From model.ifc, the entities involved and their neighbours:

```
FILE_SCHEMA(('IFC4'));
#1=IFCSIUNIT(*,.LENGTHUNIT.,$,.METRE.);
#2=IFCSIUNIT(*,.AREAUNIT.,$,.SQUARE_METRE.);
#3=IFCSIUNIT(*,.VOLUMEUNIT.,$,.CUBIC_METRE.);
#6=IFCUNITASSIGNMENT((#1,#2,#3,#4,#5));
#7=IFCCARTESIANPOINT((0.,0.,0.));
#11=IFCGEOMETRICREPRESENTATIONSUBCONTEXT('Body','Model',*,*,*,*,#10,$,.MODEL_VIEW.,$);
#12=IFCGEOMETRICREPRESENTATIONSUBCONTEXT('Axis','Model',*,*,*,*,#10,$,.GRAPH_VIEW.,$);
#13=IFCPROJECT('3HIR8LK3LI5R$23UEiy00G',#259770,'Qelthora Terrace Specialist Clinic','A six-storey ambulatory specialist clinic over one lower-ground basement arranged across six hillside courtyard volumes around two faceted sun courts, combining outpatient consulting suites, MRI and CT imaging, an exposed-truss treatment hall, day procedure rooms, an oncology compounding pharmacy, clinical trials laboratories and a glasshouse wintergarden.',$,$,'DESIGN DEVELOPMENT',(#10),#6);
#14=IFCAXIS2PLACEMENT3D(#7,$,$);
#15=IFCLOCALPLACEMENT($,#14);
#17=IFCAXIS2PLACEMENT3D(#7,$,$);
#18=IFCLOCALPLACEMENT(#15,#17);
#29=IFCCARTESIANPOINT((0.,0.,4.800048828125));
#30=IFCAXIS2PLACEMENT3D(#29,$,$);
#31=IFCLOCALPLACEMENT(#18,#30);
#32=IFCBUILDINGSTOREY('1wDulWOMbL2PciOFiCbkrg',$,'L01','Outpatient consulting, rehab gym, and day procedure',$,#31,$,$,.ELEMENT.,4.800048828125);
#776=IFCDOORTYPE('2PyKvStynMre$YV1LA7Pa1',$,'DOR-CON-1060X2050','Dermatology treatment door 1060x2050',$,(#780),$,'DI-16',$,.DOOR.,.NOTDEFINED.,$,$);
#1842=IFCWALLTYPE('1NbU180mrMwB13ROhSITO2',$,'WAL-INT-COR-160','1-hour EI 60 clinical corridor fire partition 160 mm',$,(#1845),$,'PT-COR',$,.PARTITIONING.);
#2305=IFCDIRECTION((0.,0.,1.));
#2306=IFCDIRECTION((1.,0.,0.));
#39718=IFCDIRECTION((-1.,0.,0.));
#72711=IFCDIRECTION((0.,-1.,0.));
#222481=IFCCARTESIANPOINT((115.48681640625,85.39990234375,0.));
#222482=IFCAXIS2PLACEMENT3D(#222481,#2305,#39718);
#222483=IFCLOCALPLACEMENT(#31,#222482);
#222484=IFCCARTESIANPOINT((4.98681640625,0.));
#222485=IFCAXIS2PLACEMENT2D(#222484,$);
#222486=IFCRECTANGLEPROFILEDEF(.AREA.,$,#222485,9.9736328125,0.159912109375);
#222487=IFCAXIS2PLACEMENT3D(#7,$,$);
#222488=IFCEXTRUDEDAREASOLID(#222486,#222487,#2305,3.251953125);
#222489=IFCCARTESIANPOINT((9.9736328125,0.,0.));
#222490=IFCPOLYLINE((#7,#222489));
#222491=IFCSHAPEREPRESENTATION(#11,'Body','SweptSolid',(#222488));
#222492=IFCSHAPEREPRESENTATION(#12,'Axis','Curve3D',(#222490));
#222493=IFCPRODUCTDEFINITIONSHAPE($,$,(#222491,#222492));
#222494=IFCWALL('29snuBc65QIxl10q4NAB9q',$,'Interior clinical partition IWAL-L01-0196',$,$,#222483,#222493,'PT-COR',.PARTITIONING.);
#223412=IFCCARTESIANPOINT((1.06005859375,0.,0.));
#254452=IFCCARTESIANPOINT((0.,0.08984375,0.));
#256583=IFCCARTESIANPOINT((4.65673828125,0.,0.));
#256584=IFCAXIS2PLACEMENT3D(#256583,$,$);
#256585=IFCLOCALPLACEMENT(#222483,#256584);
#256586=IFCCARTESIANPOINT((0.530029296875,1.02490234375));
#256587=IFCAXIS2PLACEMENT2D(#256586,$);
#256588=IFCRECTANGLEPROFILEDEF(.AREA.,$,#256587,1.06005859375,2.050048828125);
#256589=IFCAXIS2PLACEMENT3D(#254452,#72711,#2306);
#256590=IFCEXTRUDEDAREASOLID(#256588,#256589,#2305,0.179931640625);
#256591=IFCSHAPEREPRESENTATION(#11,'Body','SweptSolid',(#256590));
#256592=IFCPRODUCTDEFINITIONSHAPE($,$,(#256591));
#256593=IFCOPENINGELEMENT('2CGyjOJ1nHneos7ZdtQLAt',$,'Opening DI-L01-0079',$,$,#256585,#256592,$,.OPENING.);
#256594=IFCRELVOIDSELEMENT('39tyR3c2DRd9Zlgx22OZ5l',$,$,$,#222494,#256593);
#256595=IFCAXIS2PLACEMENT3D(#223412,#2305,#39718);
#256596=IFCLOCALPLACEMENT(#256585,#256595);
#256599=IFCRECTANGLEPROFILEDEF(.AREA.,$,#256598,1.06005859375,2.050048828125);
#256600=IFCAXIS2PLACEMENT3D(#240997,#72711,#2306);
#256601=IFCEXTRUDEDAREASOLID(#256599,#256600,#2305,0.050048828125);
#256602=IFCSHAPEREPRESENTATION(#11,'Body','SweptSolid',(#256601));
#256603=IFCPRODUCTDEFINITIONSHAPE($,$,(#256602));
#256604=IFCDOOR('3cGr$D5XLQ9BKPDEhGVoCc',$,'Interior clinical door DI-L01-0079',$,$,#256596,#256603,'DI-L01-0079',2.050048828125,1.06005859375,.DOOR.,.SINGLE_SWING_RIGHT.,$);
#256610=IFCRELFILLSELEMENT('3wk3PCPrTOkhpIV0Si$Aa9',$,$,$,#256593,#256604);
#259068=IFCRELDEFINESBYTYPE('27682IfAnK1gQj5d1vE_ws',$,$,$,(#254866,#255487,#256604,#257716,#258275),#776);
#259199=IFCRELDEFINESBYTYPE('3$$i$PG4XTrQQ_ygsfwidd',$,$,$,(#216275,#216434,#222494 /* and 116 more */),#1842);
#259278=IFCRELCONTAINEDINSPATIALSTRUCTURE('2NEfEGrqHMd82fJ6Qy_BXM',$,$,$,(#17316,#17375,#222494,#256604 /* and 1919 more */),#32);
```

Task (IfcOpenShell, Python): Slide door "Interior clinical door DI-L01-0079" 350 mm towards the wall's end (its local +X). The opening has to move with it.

```python
import ifcopenshell
import ifcopenshell.api.geometry
import ifcopenshell.util.placement
import ifcopenshell.util.unit

model = ifcopenshell.open("model.ifc")
unit_scale = ifcopenshell.util.unit.calculate_unit_scale(model)

door = model.by_guid("3cGr$D5XLQ9BKPDEhGVoCc")
opening = door.FillsVoids[0].RelatingOpeningElement
wall = opening.VoidsElements[0].RelatingBuildingElement

wall_matrix = ifcopenshell.util.placement.get_local_placement(wall.ObjectPlacement)
shift = wall_matrix[:3, 0] * 0.35 / unit_scale
before = ifcopenshell.util.placement.get_local_placement(door.ObjectPlacement)[:3, 3].copy()

# The door is placed relative to its opening, so it follows when the opening moves.
matrix = ifcopenshell.util.placement.get_local_placement(opening.ObjectPlacement)
matrix[:3, 3] += shift
ifcopenshell.api.geometry.edit_object_placement(
    model, product=opening, matrix=matrix, is_si=False, should_transform_children=True
)

after = ifcopenshell.util.placement.get_local_placement(door.ObjectPlacement)[:3, 3]
print("door moved by", (after - before).round(3) + 0.0)

model.write("model-out.ifc")
```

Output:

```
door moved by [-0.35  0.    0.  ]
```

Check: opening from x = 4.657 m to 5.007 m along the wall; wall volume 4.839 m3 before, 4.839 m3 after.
